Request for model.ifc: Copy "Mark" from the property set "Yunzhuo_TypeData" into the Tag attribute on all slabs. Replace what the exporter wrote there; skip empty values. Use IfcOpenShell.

First a look at what the model holds.

```python
import ifcopenshell
import ifcopenshell.util.element

model = ifcopenshell.open("model.ifc")
print(model.schema)
slabs = model.by_type("IfcSlab")
print(len(slabs), "slabs")
for e in slabs[:8]:
    source = ifcopenshell.util.element.get_pset(e, "Yunzhuo_TypeData", "Mark")
    target = e.Tag
    print(e.id(), repr(source), repr(target), sep=" | ")
```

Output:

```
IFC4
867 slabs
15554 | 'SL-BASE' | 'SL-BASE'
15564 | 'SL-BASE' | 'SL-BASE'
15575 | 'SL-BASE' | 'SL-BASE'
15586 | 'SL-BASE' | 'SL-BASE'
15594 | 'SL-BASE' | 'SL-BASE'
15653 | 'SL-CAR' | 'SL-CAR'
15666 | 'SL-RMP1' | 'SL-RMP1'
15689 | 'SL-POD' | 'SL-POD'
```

```python
import ifcopenshell
import ifcopenshell.util.element

model = ifcopenshell.open("model.ifc")

count = 0
for e in model.by_type("IfcSlab"):
    value = ifcopenshell.util.element.get_pset(e, "Yunzhuo_TypeData", "Mark")
    current = e.Tag
    if not value or not value.strip() or current == value:
        continue
    e.Tag = value
    count += 1

print(count, "slabs updated")

model.write("model_rev.ifc")
```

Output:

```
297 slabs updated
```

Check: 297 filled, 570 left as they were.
